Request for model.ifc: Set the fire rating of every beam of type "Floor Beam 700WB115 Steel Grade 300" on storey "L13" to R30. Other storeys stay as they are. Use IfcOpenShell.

First a look at what the model holds.

```python
import ifcopenshell
import ifcopenshell.util.element

model = ifcopenshell.open("model.ifc")
print(model.schema)
storey = next(s for s in model.by_type("IfcBuildingStorey") if s.Name == "L13")
beams = [e for e in ifcopenshell.util.element.get_decomposition(storey) if e.is_a("IfcBeam")]
seen = {}
for e in beams:
    element_type = ifcopenshell.util.element.get_type(e)
    key = (element_type.Name if element_type != e and element_type else None, ifcopenshell.util.element.get_pset(e, "Pset_BeamCommon", "FireRating"))
    seen[key] = seen.get(key, 0) + 1
for (name, value), count in sorted(seen.items(), key=str):
    print(count, "x", name, "|", value)
```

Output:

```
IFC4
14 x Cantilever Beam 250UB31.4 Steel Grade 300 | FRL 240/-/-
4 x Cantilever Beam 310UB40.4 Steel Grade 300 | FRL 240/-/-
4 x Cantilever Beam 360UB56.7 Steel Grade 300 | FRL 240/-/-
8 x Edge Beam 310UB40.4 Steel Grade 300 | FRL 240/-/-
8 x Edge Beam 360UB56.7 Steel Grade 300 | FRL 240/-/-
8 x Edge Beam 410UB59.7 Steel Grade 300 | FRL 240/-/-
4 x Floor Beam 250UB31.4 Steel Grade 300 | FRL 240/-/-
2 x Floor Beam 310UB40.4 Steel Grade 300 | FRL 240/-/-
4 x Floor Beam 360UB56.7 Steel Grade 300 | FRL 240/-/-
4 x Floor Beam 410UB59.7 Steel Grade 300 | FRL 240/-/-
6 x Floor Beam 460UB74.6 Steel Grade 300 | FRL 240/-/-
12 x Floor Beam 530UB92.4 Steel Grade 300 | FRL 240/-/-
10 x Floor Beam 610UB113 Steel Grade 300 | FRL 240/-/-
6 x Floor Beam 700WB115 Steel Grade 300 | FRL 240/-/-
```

```python
import ifcopenshell
import ifcopenshell.api.pset
import ifcopenshell.util.element

model = ifcopenshell.open("model.ifc")

storey = next(s for s in model.by_type("IfcBuildingStorey") if s.Name == "L13")
beams = [e for e in ifcopenshell.util.element.get_decomposition(storey) if e.is_a("IfcBeam")]

count = 0
for e in beams:
    element_type = ifcopenshell.util.element.get_type(e)
    if element_type in (None, e) or element_type.Name != "Floor Beam 700WB115 Steel Grade 300":
        continue
    found = ifcopenshell.util.element.get_pset(e, "Pset_BeamCommon", should_inherit=False)
    if found:
        pset = model.by_id(found["id"])
        if len(ifcopenshell.util.element.get_elements_by_pset(pset)) > 1:
            pset = ifcopenshell.api.pset.unshare_pset(model, products=[e], pset=pset)[0]
    else:
        pset = ifcopenshell.api.pset.add_pset(model, product=e, name="Pset_BeamCommon")
    ifcopenshell.api.pset.edit_pset(model, pset=pset, properties={"FireRating": "R30"})
    count += 1

print(count, "beams updated")

model.write("model_updated.ifc")
```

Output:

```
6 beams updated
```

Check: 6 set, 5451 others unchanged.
